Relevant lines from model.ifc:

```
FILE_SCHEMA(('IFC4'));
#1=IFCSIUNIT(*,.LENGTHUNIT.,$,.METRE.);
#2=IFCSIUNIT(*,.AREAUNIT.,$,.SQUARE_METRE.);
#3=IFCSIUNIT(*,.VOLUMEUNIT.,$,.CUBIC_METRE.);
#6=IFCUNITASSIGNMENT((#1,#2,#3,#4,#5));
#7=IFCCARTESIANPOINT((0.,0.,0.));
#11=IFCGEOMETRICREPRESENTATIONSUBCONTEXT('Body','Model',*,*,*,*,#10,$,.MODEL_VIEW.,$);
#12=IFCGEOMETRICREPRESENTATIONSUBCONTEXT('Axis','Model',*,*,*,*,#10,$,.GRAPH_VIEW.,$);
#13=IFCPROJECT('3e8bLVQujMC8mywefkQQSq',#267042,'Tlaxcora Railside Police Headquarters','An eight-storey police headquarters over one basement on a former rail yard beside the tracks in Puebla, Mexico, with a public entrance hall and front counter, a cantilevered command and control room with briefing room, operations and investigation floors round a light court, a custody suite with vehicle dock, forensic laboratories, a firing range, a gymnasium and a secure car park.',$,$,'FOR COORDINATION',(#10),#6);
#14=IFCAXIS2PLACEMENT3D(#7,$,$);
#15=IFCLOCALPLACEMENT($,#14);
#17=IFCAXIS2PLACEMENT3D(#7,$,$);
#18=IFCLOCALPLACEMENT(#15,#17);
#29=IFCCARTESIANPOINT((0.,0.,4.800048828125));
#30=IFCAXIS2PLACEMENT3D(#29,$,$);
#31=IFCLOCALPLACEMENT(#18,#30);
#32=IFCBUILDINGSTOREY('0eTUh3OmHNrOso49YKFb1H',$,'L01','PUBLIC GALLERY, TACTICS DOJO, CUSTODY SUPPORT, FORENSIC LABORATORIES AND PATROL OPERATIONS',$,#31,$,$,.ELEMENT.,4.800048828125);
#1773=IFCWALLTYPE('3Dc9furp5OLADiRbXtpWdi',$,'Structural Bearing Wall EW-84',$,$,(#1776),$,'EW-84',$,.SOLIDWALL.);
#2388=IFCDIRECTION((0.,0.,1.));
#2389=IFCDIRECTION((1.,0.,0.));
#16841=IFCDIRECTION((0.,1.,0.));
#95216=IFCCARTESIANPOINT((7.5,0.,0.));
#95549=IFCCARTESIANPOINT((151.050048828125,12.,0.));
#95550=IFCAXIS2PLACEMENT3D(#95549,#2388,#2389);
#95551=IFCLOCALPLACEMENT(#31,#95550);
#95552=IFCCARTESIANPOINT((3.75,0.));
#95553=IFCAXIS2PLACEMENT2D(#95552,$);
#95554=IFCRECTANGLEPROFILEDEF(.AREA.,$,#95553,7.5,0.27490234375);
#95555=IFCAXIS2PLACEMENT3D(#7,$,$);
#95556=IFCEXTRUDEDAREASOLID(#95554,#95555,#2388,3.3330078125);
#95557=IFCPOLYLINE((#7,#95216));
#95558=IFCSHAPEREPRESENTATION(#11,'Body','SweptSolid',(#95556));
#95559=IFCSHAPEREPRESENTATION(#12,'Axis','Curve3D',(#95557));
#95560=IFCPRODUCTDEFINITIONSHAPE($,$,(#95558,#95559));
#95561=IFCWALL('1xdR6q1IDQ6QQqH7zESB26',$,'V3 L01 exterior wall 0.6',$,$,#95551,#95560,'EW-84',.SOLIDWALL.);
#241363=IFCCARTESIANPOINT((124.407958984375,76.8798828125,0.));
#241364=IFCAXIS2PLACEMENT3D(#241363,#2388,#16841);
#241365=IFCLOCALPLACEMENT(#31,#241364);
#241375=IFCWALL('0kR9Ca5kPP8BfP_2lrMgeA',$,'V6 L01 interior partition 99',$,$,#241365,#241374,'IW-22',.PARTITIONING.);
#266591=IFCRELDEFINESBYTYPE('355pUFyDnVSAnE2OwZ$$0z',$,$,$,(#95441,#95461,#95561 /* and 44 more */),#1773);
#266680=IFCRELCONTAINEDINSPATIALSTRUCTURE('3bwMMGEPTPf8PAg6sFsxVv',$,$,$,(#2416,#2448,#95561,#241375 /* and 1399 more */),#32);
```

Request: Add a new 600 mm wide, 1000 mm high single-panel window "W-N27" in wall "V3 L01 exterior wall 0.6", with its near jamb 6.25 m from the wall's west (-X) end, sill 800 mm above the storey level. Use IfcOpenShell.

```python
import numpy as np
import ifcopenshell
import ifcopenshell.api.feature
import ifcopenshell.api.geometry
import ifcopenshell.api.root
import ifcopenshell.api.spatial
import ifcopenshell.geom
import ifcopenshell.util.element
import ifcopenshell.util.placement
import ifcopenshell.util.representation
import ifcopenshell.util.shape
import ifcopenshell.util.unit

model = ifcopenshell.open("model.ifc")
unit_scale = ifcopenshell.util.unit.calculate_unit_scale(model)
settings = ifcopenshell.geom.settings()


def volume(element):
    """Net volume in cubic metres, openings subtracted."""
    shape = ifcopenshell.geom.create_shape(settings, element)
    return ifcopenshell.util.shape.get_volume(shape.geometry)


wall = model.by_guid("1xdR6q1IDQ6QQqH7zESB26")
storey = ifcopenshell.util.element.get_container(wall, ifc_class="IfcBuildingStorey")
context = ifcopenshell.util.representation.get_context(model, "Model", "Body", "MODEL_VIEW")
before = volume(wall)

width, height, from_end, sill = 0.6, 1, 6.25, 0.8  # metres

# The wall runs along its own X axis, and the end named is its -X end.
wall_shape = ifcopenshell.geom.create_shape(settings, wall)
x, y, z = ifcopenshell.util.shape.get_vertices(wall_shape.geometry).T
start = x.min() + from_end
face, thickness = float(y.min()), float(y.max() - y.min())
wall_matrix = ifcopenshell.util.placement.get_local_placement(wall.ObjectPlacement)
level = ifcopenshell.util.placement.get_local_placement(storey.ObjectPlacement)[2, 3]


def in_wall(x, y):
    """Placement at x, y metres in the wall's axes, at sill height."""
    matrix = wall_matrix.copy()
    matrix[:, 3] = wall_matrix @ np.array([x / unit_scale, y / unit_scale, 0.0, 1.0])
    matrix[2, 3] = level + sill / unit_scale
    return matrix


# Opening: a box that overshoots both wall faces by 50 mm.
opening = ifcopenshell.api.root.create_entity(model, ifc_class="IfcOpeningElement", predefined_type="OPENING")
box = ifcopenshell.api.geometry.add_wall_representation(
    model, context=context, length=width, height=height, thickness=thickness + 0.1
)
ifcopenshell.api.geometry.assign_representation(model, product=opening, representation=box)
ifcopenshell.api.geometry.edit_object_placement(model, product=opening, matrix=in_wall(start, face - 0.05), is_si=False)
ifcopenshell.api.feature.add_feature(model, feature=opening, element=wall)

window = ifcopenshell.api.root.create_entity(model, ifc_class="IfcWindow", name="W-N27", predefined_type="WINDOW")
window.OverallWidth, window.OverallHeight = width / unit_scale, height / unit_scale
window.PartitioningType = "SINGLE_PANEL"
body = ifcopenshell.api.geometry.add_window_representation(
    model,
    context=context,
    overall_width=window.OverallWidth,
    overall_height=window.OverallHeight,
    partition_type="SINGLE_PANEL",
)
ifcopenshell.api.geometry.assign_representation(model, product=window, representation=body)
ifcopenshell.api.spatial.assign_container(model, products=[window], relating_structure=storey)
ifcopenshell.api.feature.add_filling(model, opening=opening, element=window)

# Centre the window in the wall's thickness.
ifcopenshell.api.geometry.edit_object_placement(model, product=window, matrix=in_wall(start, face), is_si=False)
window_shape = ifcopenshell.geom.create_shape(settings, window)
depth = ifcopenshell.util.shape.get_vertices(window_shape.geometry)[:, 1]
offset = face + thickness / 2 - (depth.min() + depth.max()) / 2
ifcopenshell.api.geometry.edit_object_placement(model, product=window, matrix=in_wall(start, offset), is_si=False)

after = volume(wall)

print(f"wall volume {before:.3f} -> {after:.3f} m3")

model.write("model-out.ifc")
```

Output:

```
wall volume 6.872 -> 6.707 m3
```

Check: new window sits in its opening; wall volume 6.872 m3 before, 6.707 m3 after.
